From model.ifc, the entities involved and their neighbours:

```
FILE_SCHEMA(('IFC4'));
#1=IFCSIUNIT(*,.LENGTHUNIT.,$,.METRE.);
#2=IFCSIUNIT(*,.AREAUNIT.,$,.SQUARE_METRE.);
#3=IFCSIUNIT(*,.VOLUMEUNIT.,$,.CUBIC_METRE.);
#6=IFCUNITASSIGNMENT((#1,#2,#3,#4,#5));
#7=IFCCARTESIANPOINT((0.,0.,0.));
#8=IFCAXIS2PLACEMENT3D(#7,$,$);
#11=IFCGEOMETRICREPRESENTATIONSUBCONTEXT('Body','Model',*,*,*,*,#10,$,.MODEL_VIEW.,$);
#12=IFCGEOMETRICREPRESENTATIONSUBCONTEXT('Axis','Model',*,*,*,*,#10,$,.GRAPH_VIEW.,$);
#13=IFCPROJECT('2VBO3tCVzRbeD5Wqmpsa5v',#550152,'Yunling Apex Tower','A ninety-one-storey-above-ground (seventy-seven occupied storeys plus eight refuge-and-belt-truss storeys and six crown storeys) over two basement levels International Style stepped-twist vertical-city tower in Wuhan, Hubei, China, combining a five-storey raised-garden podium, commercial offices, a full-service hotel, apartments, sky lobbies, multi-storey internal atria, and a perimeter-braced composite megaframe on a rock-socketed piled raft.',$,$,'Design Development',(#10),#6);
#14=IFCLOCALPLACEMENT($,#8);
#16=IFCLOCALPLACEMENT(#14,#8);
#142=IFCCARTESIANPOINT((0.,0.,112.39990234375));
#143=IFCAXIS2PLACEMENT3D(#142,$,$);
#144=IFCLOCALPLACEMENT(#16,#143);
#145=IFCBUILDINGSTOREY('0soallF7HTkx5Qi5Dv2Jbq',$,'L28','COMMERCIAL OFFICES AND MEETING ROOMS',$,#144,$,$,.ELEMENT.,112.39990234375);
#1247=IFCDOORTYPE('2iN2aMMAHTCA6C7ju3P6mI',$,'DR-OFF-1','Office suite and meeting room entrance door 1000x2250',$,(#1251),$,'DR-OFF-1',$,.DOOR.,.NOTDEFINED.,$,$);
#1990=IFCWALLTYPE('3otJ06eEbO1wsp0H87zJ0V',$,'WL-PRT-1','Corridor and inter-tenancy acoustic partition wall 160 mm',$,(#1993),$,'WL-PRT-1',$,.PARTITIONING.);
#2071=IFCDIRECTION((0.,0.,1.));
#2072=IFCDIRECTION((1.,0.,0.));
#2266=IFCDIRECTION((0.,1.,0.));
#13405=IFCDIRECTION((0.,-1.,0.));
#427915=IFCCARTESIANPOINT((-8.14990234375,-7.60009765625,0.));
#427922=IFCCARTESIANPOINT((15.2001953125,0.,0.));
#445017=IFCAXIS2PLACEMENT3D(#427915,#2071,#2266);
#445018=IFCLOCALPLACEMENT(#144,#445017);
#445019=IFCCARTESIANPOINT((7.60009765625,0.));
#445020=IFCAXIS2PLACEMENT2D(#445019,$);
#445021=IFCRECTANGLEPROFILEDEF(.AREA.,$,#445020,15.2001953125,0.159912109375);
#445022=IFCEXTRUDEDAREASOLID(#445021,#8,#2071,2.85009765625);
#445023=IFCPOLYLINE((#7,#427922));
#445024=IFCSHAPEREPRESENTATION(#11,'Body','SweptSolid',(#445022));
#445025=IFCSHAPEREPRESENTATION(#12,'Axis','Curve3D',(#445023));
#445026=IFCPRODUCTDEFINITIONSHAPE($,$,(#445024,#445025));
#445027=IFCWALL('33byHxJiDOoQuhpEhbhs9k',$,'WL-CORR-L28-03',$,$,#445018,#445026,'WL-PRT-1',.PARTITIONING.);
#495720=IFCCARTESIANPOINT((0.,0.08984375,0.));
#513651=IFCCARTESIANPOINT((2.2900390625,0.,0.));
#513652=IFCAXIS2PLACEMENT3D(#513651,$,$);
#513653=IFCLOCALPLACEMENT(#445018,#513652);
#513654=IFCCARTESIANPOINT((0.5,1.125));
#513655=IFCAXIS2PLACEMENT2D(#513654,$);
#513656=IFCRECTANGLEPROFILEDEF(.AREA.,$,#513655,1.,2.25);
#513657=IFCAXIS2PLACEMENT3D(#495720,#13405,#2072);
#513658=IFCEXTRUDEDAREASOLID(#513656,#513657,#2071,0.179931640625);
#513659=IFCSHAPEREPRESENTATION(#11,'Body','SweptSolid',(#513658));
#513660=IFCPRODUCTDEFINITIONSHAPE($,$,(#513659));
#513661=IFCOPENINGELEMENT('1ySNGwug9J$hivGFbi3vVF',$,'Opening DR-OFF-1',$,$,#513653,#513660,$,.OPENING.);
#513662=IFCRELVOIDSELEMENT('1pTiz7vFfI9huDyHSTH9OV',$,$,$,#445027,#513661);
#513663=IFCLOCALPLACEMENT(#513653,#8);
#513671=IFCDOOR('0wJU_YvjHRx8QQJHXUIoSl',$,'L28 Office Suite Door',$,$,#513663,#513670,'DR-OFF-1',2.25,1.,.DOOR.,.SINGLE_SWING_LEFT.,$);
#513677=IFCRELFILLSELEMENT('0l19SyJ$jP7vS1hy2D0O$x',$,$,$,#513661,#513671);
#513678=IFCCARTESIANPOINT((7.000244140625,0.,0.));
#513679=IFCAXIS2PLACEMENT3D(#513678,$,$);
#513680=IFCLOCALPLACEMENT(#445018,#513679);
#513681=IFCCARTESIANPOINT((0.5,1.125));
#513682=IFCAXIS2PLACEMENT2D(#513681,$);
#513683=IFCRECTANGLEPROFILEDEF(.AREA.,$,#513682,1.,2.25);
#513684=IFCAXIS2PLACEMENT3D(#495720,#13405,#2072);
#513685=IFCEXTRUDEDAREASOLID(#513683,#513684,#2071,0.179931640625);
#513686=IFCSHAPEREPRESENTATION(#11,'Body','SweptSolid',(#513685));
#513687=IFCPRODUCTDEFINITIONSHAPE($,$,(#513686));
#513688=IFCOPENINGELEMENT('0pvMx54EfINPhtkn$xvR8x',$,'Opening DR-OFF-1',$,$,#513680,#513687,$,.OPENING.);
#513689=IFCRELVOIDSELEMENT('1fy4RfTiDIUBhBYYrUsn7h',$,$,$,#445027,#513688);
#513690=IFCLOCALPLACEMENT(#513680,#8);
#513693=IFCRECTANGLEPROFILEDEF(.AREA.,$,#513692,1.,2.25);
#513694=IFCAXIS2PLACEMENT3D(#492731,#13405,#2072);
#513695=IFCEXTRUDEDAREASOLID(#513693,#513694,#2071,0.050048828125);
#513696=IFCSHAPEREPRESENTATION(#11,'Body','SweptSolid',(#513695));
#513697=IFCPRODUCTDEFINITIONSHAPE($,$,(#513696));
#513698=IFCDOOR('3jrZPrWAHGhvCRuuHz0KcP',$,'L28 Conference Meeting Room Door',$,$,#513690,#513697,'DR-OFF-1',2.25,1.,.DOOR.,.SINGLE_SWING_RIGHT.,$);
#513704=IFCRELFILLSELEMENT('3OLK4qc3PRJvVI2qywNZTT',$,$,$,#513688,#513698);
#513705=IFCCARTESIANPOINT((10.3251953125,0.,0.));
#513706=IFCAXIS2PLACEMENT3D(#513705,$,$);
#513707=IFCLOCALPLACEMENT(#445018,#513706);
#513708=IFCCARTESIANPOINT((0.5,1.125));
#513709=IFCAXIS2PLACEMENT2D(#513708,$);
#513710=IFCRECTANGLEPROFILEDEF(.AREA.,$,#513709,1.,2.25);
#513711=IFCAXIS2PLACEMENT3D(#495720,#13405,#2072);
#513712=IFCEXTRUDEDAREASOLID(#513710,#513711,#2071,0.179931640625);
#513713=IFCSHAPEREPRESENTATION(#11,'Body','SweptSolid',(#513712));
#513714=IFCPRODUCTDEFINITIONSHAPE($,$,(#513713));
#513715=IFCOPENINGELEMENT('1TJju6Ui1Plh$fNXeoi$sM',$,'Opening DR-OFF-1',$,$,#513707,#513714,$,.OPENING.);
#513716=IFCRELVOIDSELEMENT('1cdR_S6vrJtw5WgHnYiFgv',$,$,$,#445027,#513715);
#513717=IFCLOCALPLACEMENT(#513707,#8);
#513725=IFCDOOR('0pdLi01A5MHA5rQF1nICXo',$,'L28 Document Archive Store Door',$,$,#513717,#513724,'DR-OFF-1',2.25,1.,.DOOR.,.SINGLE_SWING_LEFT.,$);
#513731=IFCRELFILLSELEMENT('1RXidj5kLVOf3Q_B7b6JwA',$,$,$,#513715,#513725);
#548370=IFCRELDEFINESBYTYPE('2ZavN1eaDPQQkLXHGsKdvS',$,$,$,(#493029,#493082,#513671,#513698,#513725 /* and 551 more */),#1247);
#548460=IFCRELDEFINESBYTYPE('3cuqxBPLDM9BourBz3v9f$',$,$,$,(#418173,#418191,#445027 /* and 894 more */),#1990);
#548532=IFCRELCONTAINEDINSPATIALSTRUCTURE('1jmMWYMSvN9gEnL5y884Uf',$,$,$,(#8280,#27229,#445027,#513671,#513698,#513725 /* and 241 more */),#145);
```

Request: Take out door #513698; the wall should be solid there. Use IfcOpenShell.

```python
import ifcopenshell
import ifcopenshell.api.feature
import ifcopenshell.api.root
import ifcopenshell.geom
import ifcopenshell.util.shape

model = ifcopenshell.open("model.ifc")
settings = ifcopenshell.geom.settings()


def volume(element):
    """Net volume in cubic metres, openings subtracted."""
    shape = ifcopenshell.geom.create_shape(settings, element)
    return ifcopenshell.util.shape.get_volume(shape.geometry)


door = model.by_guid("3jrZPrWAHGhvCRuuHz0KcP")
opening = door.FillsVoids[0].RelatingOpeningElement
wall = opening.VoidsElements[0].RelatingBuildingElement
before = volume(wall)

ifcopenshell.api.root.remove_product(model, product=door)
ifcopenshell.api.feature.remove_feature(model, feature=opening)

after = volume(wall)

print(f"wall volume {before:.3f} -> {after:.3f} m3")

model.write("model_v2.ifc")
```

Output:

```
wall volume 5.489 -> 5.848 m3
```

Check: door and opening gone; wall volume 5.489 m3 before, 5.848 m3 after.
